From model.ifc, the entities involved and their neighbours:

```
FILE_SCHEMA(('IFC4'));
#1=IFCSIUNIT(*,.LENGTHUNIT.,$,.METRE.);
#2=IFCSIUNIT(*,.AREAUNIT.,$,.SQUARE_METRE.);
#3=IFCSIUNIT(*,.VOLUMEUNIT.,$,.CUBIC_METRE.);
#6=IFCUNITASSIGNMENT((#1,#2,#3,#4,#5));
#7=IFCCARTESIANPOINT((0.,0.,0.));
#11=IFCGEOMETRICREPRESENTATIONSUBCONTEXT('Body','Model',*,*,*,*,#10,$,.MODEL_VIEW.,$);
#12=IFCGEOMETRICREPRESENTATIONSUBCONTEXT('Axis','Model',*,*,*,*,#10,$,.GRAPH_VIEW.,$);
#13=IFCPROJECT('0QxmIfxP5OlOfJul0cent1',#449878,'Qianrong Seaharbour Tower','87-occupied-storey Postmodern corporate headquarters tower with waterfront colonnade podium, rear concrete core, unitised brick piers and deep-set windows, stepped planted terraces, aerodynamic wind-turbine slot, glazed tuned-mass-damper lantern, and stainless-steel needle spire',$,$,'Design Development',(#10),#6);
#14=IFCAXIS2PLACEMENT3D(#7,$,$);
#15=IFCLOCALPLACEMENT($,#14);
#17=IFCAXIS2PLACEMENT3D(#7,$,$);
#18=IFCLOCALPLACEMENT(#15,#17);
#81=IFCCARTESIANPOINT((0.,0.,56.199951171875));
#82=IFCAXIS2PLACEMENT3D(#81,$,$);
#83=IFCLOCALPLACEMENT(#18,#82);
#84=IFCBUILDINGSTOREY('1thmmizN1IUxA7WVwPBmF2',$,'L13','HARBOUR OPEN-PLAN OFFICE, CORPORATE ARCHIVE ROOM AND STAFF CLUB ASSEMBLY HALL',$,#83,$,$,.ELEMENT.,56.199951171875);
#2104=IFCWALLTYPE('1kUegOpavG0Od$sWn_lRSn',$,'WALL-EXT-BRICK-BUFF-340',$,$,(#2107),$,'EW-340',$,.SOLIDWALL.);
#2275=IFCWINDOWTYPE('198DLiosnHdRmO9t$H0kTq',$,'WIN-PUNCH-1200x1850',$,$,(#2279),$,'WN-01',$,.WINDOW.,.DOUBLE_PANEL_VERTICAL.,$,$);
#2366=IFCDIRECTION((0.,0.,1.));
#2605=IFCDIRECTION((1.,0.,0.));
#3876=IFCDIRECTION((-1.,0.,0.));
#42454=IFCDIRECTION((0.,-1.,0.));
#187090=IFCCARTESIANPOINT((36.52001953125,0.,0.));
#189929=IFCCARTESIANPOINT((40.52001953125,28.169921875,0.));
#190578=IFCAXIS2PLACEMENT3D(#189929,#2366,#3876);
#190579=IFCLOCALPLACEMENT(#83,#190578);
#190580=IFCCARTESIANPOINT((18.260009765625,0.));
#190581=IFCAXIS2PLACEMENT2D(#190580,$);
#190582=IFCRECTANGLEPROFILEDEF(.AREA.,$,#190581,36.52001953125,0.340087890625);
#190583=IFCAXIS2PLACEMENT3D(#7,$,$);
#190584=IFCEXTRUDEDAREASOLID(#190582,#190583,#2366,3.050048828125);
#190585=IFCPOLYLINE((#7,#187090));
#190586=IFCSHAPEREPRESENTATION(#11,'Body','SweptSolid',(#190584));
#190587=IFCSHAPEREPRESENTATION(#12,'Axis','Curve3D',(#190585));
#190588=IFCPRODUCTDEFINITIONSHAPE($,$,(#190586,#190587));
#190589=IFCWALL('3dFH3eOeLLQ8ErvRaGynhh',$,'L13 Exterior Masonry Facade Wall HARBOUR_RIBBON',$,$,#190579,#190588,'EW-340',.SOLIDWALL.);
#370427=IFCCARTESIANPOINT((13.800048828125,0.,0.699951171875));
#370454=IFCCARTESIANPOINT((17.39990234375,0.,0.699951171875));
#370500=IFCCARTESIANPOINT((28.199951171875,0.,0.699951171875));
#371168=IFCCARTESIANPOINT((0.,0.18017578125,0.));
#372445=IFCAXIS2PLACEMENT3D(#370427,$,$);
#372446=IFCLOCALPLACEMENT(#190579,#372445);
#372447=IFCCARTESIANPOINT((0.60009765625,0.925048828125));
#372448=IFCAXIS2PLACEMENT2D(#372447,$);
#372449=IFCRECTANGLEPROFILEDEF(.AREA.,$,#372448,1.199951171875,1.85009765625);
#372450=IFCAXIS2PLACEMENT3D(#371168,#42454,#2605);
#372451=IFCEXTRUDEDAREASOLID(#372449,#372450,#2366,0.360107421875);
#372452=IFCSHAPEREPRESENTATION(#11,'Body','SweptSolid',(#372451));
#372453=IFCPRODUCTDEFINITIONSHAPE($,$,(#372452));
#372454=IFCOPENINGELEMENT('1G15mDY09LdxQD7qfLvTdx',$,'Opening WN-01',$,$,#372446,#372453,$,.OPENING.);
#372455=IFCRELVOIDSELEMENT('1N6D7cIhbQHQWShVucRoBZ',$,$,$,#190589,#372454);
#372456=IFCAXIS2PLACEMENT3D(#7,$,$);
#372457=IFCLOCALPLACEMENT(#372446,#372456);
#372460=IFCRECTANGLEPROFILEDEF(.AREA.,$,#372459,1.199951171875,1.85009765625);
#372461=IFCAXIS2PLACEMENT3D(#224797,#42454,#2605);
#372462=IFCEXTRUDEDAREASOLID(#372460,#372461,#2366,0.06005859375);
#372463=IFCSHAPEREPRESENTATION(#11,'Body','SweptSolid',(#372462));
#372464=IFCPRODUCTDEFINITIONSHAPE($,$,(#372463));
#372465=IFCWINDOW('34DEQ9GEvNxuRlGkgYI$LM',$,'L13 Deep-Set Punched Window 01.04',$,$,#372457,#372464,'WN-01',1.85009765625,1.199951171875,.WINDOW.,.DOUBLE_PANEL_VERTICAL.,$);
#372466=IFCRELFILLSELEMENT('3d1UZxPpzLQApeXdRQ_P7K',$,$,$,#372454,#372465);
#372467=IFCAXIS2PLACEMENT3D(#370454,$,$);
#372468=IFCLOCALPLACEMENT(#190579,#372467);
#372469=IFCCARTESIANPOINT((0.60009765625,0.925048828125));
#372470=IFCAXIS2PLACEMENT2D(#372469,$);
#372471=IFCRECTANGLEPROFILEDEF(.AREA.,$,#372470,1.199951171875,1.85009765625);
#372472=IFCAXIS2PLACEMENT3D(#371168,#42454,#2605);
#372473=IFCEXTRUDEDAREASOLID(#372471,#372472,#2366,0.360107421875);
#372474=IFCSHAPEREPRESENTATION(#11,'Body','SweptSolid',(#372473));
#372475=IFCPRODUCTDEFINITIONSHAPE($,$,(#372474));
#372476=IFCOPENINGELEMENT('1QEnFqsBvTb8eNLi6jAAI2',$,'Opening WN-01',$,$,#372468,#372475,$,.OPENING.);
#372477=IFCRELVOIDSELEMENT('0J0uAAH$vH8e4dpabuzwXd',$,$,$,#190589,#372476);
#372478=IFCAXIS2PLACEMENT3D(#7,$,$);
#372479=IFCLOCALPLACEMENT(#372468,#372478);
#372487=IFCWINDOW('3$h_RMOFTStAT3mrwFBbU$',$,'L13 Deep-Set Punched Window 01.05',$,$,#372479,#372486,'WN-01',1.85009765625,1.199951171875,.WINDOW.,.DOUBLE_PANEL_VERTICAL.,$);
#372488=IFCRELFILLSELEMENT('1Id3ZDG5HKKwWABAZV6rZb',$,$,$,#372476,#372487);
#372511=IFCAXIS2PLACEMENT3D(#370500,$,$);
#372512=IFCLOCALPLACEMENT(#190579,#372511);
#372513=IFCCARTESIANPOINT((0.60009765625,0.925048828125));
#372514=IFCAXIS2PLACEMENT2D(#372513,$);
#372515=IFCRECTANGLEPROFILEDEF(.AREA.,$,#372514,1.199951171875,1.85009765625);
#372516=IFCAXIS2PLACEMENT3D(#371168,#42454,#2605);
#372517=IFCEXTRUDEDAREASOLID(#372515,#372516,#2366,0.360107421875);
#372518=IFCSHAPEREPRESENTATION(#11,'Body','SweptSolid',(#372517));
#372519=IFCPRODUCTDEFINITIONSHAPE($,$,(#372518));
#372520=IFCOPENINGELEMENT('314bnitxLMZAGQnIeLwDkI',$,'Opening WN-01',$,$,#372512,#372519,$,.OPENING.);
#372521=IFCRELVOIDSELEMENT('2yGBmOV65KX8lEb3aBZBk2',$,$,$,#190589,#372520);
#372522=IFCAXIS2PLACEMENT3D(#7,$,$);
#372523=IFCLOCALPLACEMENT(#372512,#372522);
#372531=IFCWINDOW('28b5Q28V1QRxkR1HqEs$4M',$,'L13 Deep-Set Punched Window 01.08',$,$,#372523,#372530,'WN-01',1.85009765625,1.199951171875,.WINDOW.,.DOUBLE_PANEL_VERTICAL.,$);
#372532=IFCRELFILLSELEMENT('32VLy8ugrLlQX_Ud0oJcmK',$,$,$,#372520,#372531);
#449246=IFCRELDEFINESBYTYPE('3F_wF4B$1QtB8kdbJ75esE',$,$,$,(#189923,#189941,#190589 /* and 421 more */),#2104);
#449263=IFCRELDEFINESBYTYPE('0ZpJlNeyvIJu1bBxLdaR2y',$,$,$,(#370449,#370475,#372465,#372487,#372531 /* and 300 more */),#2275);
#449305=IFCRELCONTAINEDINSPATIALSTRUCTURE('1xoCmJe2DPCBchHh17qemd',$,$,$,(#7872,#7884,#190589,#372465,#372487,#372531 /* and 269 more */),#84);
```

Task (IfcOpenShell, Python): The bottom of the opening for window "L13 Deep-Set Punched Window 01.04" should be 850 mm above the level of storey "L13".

```python
import numpy as np
import ifcopenshell
import ifcopenshell.api.geometry
import ifcopenshell.geom
import ifcopenshell.util.element
import ifcopenshell.util.placement
import ifcopenshell.util.shape
import ifcopenshell.util.unit

model = ifcopenshell.open("model.ifc")
unit_scale = ifcopenshell.util.unit.calculate_unit_scale(model)

window = model.by_guid("34DEQ9GEvNxuRlGkgYI$LM")
opening = window.FillsVoids[0].RelatingOpeningElement
storey = ifcopenshell.util.element.get_container(window, ifc_class="IfcBuildingStorey")
level = ifcopenshell.util.placement.get_local_placement(storey.ObjectPlacement)[2, 3]

# The opening's origin need not be at the sill, so measure its lowest point.
shape = ifcopenshell.geom.create_shape(ifcopenshell.geom.settings(), opening)
bottom = ifcopenshell.util.shape.get_shape_bottom_elevation(shape, shape.geometry) / unit_scale
dz = level + 0.85 / unit_scale - bottom

shift = np.array([0.0, 0.0, dz])
# The window is placed relative to its opening, so it follows when the opening moves.
matrix = ifcopenshell.util.placement.get_local_placement(opening.ObjectPlacement)
matrix[:3, 3] += shift
ifcopenshell.api.geometry.edit_object_placement(
    model, product=opening, matrix=matrix, is_si=False, should_transform_children=True
)

print(f"moved by {dz * unit_scale:+.3f} m")

model.write("model_updated.ifc")
```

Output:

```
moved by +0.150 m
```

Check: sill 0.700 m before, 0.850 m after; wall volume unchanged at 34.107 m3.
